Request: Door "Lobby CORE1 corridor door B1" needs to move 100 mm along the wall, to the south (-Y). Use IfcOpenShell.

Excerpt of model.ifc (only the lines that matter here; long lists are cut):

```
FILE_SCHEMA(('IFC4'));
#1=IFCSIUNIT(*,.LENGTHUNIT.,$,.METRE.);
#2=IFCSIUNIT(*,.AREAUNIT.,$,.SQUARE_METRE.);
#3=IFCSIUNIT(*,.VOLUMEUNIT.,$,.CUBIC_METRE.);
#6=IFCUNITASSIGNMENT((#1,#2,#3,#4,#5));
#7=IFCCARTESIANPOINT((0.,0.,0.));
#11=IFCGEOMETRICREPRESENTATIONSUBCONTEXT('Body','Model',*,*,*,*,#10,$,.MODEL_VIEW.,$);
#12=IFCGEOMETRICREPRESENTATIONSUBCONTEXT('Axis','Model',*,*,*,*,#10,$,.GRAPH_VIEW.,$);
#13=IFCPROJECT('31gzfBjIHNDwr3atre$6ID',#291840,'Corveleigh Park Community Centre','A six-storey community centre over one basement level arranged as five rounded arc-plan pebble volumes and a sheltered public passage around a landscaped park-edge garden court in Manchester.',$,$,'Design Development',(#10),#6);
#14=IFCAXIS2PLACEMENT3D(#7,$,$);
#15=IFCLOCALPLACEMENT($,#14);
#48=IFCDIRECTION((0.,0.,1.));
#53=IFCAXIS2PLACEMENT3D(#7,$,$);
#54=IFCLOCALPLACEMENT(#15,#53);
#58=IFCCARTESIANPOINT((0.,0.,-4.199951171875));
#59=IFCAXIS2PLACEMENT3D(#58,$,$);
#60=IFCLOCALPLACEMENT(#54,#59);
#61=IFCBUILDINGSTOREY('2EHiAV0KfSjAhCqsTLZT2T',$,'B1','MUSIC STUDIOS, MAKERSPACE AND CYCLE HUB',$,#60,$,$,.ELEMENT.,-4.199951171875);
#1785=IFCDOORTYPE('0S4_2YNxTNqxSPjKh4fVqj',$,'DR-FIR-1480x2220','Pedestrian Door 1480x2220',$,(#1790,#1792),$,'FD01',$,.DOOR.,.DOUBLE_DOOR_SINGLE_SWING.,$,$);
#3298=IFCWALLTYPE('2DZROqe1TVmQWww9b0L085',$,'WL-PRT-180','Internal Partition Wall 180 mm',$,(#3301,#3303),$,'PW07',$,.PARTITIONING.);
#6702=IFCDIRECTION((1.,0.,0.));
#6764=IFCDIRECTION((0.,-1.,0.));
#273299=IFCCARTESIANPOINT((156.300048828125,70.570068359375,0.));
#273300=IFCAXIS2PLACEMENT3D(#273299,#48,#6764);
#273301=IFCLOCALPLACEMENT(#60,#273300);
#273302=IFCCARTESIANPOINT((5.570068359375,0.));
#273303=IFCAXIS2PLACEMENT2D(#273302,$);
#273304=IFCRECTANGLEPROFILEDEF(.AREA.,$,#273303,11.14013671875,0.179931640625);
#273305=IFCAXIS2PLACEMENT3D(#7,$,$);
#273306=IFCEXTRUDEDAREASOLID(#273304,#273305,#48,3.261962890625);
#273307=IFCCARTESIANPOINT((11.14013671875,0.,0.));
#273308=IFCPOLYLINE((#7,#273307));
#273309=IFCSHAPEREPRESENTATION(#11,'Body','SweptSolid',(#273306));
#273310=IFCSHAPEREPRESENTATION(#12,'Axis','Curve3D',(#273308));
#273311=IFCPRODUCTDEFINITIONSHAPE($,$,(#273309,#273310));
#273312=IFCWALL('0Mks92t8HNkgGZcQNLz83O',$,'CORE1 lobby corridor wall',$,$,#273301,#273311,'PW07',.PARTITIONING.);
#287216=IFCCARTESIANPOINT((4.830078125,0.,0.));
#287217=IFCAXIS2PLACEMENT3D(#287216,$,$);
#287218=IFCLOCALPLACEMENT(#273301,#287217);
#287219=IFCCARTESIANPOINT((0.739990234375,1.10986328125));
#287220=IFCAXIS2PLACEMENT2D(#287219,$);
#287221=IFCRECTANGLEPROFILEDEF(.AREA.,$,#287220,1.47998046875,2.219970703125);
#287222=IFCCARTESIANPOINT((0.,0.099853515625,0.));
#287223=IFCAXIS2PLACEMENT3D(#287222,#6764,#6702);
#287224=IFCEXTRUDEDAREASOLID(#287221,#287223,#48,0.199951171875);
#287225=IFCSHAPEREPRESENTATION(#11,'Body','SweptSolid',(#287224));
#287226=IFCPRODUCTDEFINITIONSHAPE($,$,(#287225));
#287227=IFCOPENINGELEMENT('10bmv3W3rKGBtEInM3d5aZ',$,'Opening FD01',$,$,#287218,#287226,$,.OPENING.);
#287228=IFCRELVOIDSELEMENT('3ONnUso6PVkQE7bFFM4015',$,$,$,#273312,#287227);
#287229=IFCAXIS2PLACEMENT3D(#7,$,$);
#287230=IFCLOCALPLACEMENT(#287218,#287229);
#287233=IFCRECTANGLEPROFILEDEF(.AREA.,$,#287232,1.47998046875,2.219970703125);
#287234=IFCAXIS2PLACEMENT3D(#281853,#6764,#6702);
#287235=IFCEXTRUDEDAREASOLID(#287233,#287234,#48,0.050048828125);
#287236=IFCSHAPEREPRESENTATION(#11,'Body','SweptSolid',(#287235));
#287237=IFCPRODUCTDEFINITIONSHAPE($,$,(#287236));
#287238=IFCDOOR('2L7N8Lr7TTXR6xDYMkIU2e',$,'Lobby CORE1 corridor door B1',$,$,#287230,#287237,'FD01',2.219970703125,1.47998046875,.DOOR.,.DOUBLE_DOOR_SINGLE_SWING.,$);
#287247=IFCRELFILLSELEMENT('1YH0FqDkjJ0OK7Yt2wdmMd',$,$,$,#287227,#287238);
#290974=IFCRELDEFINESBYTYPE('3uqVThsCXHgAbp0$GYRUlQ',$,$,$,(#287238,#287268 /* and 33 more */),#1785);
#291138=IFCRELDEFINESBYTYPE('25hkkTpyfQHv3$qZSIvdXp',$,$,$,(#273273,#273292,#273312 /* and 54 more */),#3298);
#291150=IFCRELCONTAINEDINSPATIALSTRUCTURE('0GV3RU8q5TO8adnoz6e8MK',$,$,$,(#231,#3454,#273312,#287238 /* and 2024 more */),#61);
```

```python
import ifcopenshell
import ifcopenshell.api.geometry
import ifcopenshell.util.placement

model = ifcopenshell.open("model.ifc")

door = model.by_guid("2L7N8Lr7TTXR6xDYMkIU2e")
opening = door.FillsVoids[0].RelatingOpeningElement
wall = opening.VoidsElements[0].RelatingBuildingElement

wall_matrix = ifcopenshell.util.placement.get_local_placement(wall.ObjectPlacement)
shift = wall_matrix[:3, 0] * 0.1
before = ifcopenshell.util.placement.get_local_placement(door.ObjectPlacement)[:3, 3].copy()

# The door is placed relative to its opening, so it follows when the opening moves.
matrix = ifcopenshell.util.placement.get_local_placement(opening.ObjectPlacement)
matrix[:3, 3] += shift
ifcopenshell.api.geometry.edit_object_placement(
    model, product=opening, matrix=matrix, is_si=False, should_transform_children=True
)

after = ifcopenshell.util.placement.get_local_placement(door.ObjectPlacement)[:3, 3]
print("door moved by", (after - before).round(3) + 0.0)

model.write("model_v2.ifc")
```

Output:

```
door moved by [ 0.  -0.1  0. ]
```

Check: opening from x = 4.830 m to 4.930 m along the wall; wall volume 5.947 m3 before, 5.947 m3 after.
